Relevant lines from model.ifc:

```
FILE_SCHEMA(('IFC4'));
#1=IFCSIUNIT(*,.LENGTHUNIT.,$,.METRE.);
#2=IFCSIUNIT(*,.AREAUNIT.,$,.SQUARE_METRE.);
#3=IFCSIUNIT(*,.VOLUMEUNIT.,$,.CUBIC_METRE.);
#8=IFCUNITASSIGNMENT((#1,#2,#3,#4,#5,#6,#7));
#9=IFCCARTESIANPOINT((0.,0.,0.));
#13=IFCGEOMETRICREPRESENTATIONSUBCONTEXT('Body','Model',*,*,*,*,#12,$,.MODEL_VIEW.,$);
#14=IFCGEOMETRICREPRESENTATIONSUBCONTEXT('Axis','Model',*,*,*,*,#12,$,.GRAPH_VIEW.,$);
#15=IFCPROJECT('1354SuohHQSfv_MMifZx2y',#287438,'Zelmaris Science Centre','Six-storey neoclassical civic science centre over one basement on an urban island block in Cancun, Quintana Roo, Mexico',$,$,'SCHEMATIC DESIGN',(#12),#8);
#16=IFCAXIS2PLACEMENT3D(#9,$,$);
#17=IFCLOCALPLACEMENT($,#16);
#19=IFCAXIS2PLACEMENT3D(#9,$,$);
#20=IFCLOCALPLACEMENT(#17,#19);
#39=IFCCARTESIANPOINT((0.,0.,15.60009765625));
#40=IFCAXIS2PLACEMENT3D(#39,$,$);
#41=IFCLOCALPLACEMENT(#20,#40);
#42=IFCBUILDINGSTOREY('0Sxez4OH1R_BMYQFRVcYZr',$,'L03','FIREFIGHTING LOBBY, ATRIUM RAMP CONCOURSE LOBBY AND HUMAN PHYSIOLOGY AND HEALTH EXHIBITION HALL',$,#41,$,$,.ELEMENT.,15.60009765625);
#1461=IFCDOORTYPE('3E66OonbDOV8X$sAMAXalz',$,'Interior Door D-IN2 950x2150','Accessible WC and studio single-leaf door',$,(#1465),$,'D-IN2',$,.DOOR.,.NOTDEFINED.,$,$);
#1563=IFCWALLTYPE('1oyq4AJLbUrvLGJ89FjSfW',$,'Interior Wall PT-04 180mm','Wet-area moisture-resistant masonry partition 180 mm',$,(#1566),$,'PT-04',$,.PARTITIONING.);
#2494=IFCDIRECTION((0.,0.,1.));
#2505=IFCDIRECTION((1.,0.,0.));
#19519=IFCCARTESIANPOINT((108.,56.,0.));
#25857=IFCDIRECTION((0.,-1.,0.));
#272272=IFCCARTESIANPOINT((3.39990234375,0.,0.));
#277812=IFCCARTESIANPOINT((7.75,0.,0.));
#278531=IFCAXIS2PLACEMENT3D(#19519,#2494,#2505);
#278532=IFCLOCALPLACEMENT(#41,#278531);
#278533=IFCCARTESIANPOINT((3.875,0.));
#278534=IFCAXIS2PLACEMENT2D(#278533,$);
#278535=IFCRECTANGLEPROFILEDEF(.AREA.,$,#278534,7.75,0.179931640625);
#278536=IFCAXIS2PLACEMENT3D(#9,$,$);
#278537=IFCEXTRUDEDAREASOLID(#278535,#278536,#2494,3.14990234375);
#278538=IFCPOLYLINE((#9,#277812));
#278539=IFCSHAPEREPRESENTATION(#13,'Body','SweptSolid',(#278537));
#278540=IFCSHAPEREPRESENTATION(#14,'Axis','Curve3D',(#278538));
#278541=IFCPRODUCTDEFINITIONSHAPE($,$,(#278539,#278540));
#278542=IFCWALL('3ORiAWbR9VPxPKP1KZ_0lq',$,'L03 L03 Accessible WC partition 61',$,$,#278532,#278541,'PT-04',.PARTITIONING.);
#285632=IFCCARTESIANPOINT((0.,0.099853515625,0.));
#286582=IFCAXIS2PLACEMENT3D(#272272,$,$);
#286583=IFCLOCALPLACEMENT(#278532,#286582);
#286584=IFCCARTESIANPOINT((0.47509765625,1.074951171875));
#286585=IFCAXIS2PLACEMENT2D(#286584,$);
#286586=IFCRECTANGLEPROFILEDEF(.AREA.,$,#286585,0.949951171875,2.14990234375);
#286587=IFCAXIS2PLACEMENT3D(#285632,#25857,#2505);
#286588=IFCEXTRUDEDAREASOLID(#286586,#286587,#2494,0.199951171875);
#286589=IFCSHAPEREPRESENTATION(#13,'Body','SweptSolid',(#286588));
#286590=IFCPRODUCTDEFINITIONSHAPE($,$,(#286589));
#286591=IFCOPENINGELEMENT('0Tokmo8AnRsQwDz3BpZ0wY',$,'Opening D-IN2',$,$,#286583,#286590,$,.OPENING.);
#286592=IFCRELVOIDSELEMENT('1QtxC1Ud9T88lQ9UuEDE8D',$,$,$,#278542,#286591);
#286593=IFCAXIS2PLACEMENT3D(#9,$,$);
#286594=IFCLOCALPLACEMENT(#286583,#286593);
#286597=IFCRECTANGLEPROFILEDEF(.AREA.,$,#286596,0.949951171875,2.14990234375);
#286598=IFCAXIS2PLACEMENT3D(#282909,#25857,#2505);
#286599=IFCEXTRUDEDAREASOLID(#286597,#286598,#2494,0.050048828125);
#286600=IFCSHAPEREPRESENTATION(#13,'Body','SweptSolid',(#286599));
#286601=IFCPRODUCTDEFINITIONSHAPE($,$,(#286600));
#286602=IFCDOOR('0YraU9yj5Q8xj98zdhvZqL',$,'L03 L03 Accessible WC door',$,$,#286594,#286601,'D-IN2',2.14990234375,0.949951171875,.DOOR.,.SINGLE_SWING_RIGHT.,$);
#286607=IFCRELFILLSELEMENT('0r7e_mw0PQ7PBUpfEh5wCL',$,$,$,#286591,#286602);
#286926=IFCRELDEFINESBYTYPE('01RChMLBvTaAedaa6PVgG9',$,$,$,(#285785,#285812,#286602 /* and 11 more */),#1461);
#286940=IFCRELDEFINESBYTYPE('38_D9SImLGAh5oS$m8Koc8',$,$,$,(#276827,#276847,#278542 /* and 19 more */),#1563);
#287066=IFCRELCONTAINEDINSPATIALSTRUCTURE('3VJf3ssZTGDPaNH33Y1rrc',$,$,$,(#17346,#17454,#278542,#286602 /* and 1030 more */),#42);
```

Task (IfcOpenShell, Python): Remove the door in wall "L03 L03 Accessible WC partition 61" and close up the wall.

```python
import ifcopenshell
import ifcopenshell.api.feature
import ifcopenshell.api.root
import ifcopenshell.geom
import ifcopenshell.util.shape

model = ifcopenshell.open("model.ifc")
settings = ifcopenshell.geom.settings()


def volume(element):
    """Net volume in cubic metres, openings subtracted."""
    shape = ifcopenshell.geom.create_shape(settings, element)
    return ifcopenshell.util.shape.get_volume(shape.geometry)


door = model.by_guid("0YraU9yj5Q8xj98zdhvZqL")
opening = door.FillsVoids[0].RelatingOpeningElement
wall = opening.VoidsElements[0].RelatingBuildingElement
before = volume(wall)

ifcopenshell.api.root.remove_product(model, product=door)
ifcopenshell.api.feature.remove_feature(model, feature=opening)

after = volume(wall)

print(f"wall volume {before:.3f} -> {after:.3f} m3")

model.write("model-out.ifc")
```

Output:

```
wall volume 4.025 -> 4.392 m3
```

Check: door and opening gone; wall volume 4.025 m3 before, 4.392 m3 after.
